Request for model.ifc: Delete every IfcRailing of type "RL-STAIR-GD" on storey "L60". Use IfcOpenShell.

First a look at what the model holds.

```python
import ifcopenshell
import ifcopenshell.util.element

model = ifcopenshell.open("model.ifc")
print(model.schema)
storey = next(s for s in model.by_type("IfcBuildingStorey") if s.Name == "L60")
railings = [e for e in ifcopenshell.util.element.get_decomposition(storey) if e.is_a("IfcRailing")]
seen = {}
for e in railings:
    element_type = ifcopenshell.util.element.get_type(e)
    name = element_type.Name if element_type not in (None, e) else None
    seen[name] = seen.get(name, 0) + 1
for name, count in sorted(seen.items(), key=str):
    print(count, "x", name)
```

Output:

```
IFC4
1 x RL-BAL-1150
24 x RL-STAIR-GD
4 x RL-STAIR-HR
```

```python
import ifcopenshell
import ifcopenshell.api.root
import ifcopenshell.util.element

model = ifcopenshell.open("model.ifc")

storey = next(s for s in model.by_type("IfcBuildingStorey") if s.Name == "L60")
railings = [e for e in ifcopenshell.util.element.get_decomposition(storey) if e.is_a("IfcRailing")]
targets = [e for e in railings if (t := ifcopenshell.util.element.get_type(e)) not in (None, e) and t.Name == "RL-STAIR-GD"]

for e in targets:
    ifcopenshell.api.root.remove_product(model, product=e)
print(len(targets), "removed")

model.write("model-out.ifc")
```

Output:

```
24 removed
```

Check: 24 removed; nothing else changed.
